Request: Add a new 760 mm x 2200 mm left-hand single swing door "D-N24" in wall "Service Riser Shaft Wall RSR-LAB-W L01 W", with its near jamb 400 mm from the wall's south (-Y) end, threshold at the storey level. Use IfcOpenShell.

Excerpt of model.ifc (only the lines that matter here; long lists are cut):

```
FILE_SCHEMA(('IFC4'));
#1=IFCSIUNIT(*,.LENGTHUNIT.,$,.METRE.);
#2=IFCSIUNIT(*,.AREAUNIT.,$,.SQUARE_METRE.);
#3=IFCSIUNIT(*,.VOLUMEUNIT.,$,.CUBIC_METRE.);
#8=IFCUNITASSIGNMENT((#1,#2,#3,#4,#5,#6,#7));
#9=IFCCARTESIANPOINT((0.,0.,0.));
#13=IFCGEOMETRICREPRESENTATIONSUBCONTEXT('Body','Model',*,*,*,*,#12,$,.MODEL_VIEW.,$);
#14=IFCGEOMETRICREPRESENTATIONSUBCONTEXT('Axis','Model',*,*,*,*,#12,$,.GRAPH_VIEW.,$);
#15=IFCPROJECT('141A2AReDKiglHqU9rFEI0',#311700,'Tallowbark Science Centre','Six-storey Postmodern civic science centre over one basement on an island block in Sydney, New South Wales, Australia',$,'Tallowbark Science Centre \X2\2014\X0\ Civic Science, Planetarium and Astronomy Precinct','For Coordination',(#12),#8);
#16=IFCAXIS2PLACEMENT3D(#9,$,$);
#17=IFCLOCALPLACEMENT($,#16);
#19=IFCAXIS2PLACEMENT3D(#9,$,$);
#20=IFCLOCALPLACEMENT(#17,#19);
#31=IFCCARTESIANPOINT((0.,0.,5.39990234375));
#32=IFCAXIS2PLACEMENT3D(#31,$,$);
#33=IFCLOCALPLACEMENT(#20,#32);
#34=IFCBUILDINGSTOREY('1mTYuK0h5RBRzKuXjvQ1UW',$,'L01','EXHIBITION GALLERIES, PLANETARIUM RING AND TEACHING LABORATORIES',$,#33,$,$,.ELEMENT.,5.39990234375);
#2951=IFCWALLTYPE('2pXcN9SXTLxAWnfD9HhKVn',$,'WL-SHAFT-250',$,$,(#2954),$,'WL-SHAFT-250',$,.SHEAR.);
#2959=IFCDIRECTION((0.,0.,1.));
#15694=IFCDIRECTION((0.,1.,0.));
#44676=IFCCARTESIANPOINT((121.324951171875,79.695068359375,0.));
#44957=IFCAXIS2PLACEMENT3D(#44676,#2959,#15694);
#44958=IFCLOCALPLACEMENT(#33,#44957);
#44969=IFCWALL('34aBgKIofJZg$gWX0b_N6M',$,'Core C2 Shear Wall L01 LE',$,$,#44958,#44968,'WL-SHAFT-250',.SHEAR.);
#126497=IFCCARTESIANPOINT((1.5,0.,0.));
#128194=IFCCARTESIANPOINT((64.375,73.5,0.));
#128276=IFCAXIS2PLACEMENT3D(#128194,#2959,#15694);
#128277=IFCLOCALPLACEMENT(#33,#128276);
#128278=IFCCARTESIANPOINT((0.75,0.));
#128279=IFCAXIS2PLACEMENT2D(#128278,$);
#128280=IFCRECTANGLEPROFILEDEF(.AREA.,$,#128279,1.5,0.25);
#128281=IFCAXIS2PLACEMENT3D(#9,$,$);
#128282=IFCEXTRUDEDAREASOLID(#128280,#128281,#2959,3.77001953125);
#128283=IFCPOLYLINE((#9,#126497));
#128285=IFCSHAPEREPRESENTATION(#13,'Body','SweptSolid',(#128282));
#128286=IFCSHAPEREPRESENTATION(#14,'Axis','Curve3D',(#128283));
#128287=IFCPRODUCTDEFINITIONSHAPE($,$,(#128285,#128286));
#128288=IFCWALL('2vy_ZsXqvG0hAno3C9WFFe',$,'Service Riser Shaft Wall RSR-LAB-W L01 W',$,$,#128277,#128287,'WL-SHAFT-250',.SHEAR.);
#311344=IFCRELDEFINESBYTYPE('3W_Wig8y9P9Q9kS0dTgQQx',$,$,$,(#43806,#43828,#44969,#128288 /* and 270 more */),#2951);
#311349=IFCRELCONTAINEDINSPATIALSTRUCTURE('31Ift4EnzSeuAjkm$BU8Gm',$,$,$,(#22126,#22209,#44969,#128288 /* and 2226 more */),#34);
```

```python
import numpy as np
import ifcopenshell
import ifcopenshell.api.feature
import ifcopenshell.api.geometry
import ifcopenshell.api.root
import ifcopenshell.api.spatial
import ifcopenshell.geom
import ifcopenshell.util.element
import ifcopenshell.util.placement
import ifcopenshell.util.representation
import ifcopenshell.util.shape
import ifcopenshell.util.unit

model = ifcopenshell.open("model.ifc")
unit_scale = ifcopenshell.util.unit.calculate_unit_scale(model)
settings = ifcopenshell.geom.settings()


def volume(element):
    """Net volume in cubic metres, openings subtracted."""
    shape = ifcopenshell.geom.create_shape(settings, element)
    return ifcopenshell.util.shape.get_volume(shape.geometry)


wall = model.by_guid("2vy_ZsXqvG0hAno3C9WFFe")
storey = ifcopenshell.util.element.get_container(wall, ifc_class="IfcBuildingStorey")
context = ifcopenshell.util.representation.get_context(model, "Model", "Body", "MODEL_VIEW")
before = volume(wall)

width, height, from_end, sill = 0.76, 2.2, 0.4, 0.0  # metres

# The wall runs along its own X axis, and the end named is its -X end.
wall_shape = ifcopenshell.geom.create_shape(settings, wall)
x, y, z = ifcopenshell.util.shape.get_vertices(wall_shape.geometry).T
start = x.min() + from_end
face, thickness = float(y.min()), float(y.max() - y.min())
wall_matrix = ifcopenshell.util.placement.get_local_placement(wall.ObjectPlacement)
level = ifcopenshell.util.placement.get_local_placement(storey.ObjectPlacement)[2, 3]


def in_wall(x, y):
    """Placement at x, y metres in the wall's axes, at sill height."""
    matrix = wall_matrix.copy()
    matrix[:, 3] = wall_matrix @ np.array([x / unit_scale, y / unit_scale, 0.0, 1.0])
    matrix[2, 3] = level + sill / unit_scale
    return matrix


# Opening: a box that overshoots both wall faces by 50 mm.
opening = ifcopenshell.api.root.create_entity(model, ifc_class="IfcOpeningElement", predefined_type="OPENING")
box = ifcopenshell.api.geometry.add_wall_representation(
    model, context=context, length=width, height=height, thickness=thickness + 0.1
)
ifcopenshell.api.geometry.assign_representation(model, product=opening, representation=box)
ifcopenshell.api.geometry.edit_object_placement(model, product=opening, matrix=in_wall(start, face - 0.05), is_si=False)
ifcopenshell.api.feature.add_feature(model, feature=opening, element=wall)

door = ifcopenshell.api.root.create_entity(model, ifc_class="IfcDoor", name="D-N24", predefined_type="DOOR")
door.OverallWidth, door.OverallHeight = width / unit_scale, height / unit_scale
door.OperationType = "SINGLE_SWING_LEFT"
body = ifcopenshell.api.geometry.add_door_representation(
    model,
    context=context,
    overall_width=door.OverallWidth,
    overall_height=door.OverallHeight,
    operation_type="SINGLE_SWING_LEFT",
    lining_properties={"LiningDepth": thickness / unit_scale, "ThresholdDepth": thickness / unit_scale},
)
ifcopenshell.api.geometry.assign_representation(model, product=door, representation=body)
ifcopenshell.api.spatial.assign_container(model, products=[door], relating_structure=storey)
ifcopenshell.api.feature.add_filling(model, opening=opening, element=door)

# The lining spans the wall, so the door starts at the wall face.
ifcopenshell.api.geometry.edit_object_placement(model, product=door, matrix=in_wall(start, face), is_si=False)

after = volume(wall)

print(f"wall volume {before:.3f} -> {after:.3f} m3")

model.write("model-out.ifc")
```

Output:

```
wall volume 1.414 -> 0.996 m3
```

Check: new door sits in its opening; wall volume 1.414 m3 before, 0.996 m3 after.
